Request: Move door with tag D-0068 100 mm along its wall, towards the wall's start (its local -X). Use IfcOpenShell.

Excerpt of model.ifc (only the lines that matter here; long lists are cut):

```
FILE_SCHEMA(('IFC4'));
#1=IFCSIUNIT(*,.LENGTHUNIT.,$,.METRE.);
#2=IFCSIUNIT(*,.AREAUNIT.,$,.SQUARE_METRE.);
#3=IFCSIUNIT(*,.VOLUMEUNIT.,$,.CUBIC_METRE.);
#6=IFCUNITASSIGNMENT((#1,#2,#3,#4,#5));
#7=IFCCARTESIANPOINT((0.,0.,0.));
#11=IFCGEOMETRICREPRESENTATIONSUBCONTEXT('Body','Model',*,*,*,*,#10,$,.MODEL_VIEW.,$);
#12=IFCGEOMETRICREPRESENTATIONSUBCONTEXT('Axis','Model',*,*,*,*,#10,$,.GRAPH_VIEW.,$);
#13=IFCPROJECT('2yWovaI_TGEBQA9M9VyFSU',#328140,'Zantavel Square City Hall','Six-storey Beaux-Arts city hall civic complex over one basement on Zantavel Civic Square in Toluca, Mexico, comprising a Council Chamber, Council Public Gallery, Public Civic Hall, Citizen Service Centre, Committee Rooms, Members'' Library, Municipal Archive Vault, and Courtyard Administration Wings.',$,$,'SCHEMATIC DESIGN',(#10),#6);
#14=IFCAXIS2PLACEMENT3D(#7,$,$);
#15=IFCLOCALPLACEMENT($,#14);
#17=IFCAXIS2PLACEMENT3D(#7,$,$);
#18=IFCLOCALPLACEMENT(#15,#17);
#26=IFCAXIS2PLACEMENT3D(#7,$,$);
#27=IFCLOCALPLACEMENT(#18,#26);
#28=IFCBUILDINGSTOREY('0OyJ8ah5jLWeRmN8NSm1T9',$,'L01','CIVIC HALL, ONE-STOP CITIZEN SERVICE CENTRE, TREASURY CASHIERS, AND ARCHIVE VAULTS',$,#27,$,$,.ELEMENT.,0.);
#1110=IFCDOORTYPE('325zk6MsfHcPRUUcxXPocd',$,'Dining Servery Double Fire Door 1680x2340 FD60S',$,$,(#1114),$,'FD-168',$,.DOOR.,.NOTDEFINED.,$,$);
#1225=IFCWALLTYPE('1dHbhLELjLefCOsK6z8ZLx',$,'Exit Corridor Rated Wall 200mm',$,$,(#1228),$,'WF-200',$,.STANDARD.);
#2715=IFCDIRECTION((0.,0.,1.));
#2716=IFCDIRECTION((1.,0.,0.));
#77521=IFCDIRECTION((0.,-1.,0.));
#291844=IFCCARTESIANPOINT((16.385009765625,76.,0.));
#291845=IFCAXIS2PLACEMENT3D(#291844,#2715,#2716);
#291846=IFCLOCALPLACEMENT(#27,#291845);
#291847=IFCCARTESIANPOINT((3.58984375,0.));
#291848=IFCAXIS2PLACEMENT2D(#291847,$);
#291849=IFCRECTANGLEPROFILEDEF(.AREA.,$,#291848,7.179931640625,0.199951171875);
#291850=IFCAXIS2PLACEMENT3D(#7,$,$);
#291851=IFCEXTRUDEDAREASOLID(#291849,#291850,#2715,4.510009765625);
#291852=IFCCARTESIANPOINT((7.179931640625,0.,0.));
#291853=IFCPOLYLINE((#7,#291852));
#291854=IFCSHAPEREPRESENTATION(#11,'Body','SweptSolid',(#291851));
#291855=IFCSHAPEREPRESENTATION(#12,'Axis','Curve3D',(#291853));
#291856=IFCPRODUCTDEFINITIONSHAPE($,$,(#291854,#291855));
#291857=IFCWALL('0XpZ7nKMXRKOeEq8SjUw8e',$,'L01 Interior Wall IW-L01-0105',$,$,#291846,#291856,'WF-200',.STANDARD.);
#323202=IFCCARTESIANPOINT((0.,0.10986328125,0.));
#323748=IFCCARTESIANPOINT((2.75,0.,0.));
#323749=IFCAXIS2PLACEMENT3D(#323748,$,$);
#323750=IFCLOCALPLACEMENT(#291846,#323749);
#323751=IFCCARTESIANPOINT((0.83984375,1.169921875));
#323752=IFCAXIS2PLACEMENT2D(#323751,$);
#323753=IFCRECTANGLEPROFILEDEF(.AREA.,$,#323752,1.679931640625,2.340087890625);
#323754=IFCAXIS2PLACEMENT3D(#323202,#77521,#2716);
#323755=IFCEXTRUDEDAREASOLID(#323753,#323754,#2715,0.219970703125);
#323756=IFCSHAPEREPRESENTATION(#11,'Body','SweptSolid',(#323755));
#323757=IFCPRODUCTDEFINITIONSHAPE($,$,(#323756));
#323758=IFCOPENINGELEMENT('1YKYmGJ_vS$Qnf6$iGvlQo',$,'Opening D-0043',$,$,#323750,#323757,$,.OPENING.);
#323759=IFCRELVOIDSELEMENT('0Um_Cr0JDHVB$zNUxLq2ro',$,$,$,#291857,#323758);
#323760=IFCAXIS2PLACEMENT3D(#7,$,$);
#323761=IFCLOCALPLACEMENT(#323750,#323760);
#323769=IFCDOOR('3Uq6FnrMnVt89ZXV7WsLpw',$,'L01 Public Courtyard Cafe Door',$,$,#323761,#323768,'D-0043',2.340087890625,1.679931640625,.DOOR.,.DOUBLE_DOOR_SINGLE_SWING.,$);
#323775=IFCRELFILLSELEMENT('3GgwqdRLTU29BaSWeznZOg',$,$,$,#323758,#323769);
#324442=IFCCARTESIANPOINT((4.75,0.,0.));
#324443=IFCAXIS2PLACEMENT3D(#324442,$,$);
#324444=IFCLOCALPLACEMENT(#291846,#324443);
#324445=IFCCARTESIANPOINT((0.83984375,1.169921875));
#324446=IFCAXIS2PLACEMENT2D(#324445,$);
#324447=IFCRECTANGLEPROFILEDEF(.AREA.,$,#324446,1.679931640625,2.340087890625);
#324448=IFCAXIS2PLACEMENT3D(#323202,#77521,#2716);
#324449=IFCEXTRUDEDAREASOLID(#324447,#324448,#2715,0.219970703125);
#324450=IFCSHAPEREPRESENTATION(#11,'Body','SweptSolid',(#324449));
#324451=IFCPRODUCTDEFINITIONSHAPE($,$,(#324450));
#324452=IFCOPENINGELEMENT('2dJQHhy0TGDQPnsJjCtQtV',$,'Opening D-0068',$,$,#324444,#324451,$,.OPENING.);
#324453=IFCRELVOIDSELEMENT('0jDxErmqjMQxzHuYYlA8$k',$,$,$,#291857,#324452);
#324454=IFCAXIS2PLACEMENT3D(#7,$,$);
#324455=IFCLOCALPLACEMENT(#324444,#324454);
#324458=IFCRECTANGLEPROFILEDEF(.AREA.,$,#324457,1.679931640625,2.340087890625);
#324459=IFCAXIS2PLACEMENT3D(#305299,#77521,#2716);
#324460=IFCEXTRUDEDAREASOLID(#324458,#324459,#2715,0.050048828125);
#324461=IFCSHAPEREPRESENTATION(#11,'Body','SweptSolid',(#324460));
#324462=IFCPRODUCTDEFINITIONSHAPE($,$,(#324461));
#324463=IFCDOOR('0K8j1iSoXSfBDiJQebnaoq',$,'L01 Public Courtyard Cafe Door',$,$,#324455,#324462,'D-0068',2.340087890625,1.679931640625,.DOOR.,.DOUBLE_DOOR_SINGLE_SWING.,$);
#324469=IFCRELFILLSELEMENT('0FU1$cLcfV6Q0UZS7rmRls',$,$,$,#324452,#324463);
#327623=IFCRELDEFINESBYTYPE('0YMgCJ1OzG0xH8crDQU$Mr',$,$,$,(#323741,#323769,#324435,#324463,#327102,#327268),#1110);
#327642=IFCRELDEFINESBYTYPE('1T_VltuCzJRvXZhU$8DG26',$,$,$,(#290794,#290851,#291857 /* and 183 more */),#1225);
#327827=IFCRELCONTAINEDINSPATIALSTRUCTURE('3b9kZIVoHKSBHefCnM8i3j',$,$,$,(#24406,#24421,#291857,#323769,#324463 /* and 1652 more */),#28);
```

```python
import ifcopenshell
import ifcopenshell.api.geometry
import ifcopenshell.util.placement

model = ifcopenshell.open("model.ifc")

door = model.by_id(324463)
opening = door.FillsVoids[0].RelatingOpeningElement
wall = opening.VoidsElements[0].RelatingBuildingElement

wall_matrix = ifcopenshell.util.placement.get_local_placement(wall.ObjectPlacement)
shift = wall_matrix[:3, 0] * -0.1
before = ifcopenshell.util.placement.get_local_placement(door.ObjectPlacement)[:3, 3].copy()

# The door is placed relative to its opening, so it follows when the opening moves.
matrix = ifcopenshell.util.placement.get_local_placement(opening.ObjectPlacement)
matrix[:3, 3] += shift
ifcopenshell.api.geometry.edit_object_placement(
    model, product=opening, matrix=matrix, is_si=False, should_transform_children=True
)

after = ifcopenshell.util.placement.get_local_placement(door.ObjectPlacement)[:3, 3]
print("door moved by", (after - before).round(3) + 0.0)

model.write("model_updated.ifc")
```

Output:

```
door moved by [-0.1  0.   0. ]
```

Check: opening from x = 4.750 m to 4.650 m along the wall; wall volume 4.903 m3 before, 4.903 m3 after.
